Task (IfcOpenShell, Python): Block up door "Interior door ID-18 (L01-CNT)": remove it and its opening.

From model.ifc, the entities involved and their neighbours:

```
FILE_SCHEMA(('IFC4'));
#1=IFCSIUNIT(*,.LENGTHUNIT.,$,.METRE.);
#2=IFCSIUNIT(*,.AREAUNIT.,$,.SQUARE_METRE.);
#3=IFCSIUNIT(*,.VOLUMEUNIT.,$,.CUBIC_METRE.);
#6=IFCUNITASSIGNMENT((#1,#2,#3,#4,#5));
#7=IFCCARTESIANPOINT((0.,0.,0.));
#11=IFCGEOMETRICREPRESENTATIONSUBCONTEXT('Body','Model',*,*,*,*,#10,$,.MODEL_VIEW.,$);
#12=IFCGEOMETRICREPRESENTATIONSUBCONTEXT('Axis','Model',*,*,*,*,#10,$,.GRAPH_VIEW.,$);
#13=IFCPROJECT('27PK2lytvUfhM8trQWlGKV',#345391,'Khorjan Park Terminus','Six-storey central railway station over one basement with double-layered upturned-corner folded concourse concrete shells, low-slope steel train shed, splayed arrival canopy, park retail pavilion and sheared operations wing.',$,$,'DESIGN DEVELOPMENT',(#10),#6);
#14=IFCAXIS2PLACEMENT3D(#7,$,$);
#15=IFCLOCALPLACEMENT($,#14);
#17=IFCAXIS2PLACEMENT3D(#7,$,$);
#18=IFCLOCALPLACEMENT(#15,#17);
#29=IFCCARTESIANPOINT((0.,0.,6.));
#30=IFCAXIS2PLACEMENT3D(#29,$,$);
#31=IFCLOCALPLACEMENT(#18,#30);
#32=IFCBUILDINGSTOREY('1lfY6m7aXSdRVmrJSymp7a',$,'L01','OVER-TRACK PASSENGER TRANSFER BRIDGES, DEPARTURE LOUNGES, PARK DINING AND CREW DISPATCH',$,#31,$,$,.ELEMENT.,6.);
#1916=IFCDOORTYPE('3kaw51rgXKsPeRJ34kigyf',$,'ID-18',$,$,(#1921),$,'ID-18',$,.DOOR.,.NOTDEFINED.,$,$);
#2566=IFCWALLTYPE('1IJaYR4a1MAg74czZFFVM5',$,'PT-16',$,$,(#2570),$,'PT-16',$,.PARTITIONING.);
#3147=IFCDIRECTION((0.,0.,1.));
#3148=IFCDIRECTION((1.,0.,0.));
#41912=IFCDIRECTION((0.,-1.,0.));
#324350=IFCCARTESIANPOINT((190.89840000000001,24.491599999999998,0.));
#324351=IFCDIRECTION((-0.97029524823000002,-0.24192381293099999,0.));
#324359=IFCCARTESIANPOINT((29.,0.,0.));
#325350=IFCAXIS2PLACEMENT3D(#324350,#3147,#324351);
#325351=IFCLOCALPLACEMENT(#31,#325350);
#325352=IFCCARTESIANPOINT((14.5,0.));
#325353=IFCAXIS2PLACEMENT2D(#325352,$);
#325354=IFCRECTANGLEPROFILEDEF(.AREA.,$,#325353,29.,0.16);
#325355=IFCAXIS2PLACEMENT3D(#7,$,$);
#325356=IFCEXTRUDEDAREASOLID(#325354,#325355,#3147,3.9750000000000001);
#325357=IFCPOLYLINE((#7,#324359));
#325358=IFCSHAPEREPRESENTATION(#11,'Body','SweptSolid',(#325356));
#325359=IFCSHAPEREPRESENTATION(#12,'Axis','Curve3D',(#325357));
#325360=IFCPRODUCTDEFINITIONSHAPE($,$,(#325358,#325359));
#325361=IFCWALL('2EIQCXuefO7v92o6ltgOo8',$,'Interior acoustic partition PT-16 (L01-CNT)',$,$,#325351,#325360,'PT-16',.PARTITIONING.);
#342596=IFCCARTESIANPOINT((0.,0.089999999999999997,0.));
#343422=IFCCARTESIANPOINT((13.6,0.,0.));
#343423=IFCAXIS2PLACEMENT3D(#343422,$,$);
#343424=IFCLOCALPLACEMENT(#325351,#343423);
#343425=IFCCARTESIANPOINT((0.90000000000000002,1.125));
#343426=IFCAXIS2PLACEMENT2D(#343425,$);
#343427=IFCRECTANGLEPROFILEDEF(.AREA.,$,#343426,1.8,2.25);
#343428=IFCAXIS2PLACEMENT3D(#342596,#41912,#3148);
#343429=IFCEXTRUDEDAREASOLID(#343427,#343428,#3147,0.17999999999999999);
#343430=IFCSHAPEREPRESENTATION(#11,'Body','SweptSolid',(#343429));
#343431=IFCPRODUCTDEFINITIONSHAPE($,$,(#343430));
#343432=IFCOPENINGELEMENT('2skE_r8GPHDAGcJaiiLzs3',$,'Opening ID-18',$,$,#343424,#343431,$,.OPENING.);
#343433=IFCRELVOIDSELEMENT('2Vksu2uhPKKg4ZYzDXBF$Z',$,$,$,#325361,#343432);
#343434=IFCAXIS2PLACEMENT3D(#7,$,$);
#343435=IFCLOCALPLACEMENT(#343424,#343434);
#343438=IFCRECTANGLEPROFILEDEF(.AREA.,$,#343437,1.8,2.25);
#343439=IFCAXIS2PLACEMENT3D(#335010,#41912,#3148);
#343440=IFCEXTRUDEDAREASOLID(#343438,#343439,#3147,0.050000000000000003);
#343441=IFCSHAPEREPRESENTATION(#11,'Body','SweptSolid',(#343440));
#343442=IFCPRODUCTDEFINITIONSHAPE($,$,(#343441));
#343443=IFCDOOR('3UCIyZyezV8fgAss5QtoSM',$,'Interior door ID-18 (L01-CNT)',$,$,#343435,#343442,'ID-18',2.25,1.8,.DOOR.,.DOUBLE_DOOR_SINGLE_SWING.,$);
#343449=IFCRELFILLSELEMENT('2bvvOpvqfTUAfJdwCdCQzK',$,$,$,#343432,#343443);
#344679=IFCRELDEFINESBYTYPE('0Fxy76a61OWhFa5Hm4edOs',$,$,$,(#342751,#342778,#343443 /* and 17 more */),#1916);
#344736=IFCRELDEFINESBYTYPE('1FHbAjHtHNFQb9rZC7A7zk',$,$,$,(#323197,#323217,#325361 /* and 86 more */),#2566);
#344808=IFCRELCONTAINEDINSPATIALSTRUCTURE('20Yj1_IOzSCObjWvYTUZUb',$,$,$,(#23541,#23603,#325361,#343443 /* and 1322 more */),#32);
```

```python
import ifcopenshell
import ifcopenshell.api.feature
import ifcopenshell.api.root
import ifcopenshell.geom
import ifcopenshell.util.shape

model = ifcopenshell.open("model.ifc")
settings = ifcopenshell.geom.settings()


def volume(element):
    """Net volume in cubic metres, openings subtracted."""
    shape = ifcopenshell.geom.create_shape(settings, element)
    return ifcopenshell.util.shape.get_volume(shape.geometry)


door = model.by_guid("3UCIyZyezV8fgAss5QtoSM")
opening = door.FillsVoids[0].RelatingOpeningElement
wall = opening.VoidsElements[0].RelatingBuildingElement
before = volume(wall)

ifcopenshell.api.root.remove_product(model, product=door)
ifcopenshell.api.feature.remove_feature(model, feature=opening)

after = volume(wall)

print(f"wall volume {before:.3f} -> {after:.3f} m3")

model.write("model_updated.ifc")
```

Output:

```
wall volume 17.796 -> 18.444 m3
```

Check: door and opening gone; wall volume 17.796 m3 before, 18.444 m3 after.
